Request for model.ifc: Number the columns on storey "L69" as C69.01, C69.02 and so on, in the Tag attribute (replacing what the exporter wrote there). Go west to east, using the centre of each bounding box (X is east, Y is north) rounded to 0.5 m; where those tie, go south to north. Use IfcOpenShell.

First a look at what the model holds.

```python
import ifcopenshell
import ifcopenshell.util.element
import ifcopenshell.util.placement

model = ifcopenshell.open("model.ifc")
print(model.schema)
storey = next(s for s in model.by_type("IfcBuildingStorey") if s.Name == "L69")
columns = [e for e in ifcopenshell.util.element.get_decomposition(storey) if e.is_a("IfcColumn")]
for e in sorted(columns, key=lambda e: e.id()):
    origin = ifcopenshell.util.placement.get_local_placement(e.ObjectPlacement)[:3, 3]
    print(e.id(), e.Tag, e.Name, origin.round(2) + 0.0, sep=" | ")
```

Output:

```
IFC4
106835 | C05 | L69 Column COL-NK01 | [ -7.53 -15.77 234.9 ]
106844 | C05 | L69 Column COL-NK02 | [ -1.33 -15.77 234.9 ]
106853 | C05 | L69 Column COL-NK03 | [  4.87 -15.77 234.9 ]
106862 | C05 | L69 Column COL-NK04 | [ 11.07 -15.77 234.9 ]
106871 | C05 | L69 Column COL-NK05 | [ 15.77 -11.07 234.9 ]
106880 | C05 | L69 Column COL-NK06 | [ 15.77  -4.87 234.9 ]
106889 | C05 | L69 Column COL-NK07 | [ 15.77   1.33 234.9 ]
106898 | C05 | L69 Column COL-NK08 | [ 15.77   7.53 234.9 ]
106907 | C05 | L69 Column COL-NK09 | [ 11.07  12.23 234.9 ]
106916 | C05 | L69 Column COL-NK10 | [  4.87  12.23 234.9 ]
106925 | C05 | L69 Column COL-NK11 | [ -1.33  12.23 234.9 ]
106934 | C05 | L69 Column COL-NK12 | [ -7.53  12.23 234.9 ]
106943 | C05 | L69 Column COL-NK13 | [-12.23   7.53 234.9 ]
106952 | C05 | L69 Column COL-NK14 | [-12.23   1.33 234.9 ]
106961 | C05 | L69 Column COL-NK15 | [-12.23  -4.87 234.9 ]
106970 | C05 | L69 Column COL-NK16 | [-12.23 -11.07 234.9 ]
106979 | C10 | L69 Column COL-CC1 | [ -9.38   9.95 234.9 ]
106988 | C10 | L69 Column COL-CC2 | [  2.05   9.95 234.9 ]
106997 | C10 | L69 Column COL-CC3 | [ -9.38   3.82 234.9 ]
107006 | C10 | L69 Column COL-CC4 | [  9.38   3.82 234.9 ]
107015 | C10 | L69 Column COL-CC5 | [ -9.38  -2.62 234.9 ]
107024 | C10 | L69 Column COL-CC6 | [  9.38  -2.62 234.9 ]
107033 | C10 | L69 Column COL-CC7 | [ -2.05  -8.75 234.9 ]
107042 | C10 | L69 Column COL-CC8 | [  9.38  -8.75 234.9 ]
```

```python
import ifcopenshell
import ifcopenshell.geom
import ifcopenshell.util.element
import ifcopenshell.util.shape

model = ifcopenshell.open("model.ifc")
settings = ifcopenshell.geom.settings()
settings.set("use-world-coords", True)


def centre(element):
    shape = ifcopenshell.geom.create_shape(settings, element)
    return ifcopenshell.util.shape.get_bbox_centroid(shape.geometry)


storey = next(s for s in model.by_type("IfcBuildingStorey") if s.Name == "L69")
columns = [e for e in ifcopenshell.util.element.get_decomposition(storey) if e.is_a("IfcColumn")]

# Insertion points can sit at a corner or the storey origin, so sort by the geometry (in metres).
centres = {e: centre(e) for e in columns}
columns.sort(key=lambda e: (round(centres[e][0] / 0.5), centres[e][1]))

for i, e in enumerate(columns, start=1):
    number = f"C69.{i:02d}"
    e.Tag = number
    print(e.id(), number)

model.write("model-out.ifc")
```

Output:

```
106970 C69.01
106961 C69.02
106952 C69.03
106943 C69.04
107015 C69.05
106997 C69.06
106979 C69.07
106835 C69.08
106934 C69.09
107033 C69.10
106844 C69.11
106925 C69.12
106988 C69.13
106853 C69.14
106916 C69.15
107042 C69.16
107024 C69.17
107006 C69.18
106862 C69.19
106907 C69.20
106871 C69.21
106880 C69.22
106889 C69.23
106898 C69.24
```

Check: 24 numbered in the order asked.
